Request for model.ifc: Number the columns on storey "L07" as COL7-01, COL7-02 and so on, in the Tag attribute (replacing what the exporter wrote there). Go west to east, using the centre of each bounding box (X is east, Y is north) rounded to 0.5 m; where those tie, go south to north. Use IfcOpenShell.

First a look at what the model holds.

```python
import ifcopenshell
import ifcopenshell.util.element
import ifcopenshell.util.placement

model = ifcopenshell.open("model.ifc")
print(model.schema)
storey = next(s for s in model.by_type("IfcBuildingStorey") if s.Name == "L07")
columns = [e for e in ifcopenshell.util.element.get_decomposition(storey) if e.is_a("IfcColumn")]
for e in sorted(columns, key=lambda e: e.id()):
    origin = ifcopenshell.util.placement.get_local_placement(e.ObjectPlacement)[:3, 3]
    print(e.id(), e.Tag, e.Name, origin.round(2) + 0.0, sep=" | ")
```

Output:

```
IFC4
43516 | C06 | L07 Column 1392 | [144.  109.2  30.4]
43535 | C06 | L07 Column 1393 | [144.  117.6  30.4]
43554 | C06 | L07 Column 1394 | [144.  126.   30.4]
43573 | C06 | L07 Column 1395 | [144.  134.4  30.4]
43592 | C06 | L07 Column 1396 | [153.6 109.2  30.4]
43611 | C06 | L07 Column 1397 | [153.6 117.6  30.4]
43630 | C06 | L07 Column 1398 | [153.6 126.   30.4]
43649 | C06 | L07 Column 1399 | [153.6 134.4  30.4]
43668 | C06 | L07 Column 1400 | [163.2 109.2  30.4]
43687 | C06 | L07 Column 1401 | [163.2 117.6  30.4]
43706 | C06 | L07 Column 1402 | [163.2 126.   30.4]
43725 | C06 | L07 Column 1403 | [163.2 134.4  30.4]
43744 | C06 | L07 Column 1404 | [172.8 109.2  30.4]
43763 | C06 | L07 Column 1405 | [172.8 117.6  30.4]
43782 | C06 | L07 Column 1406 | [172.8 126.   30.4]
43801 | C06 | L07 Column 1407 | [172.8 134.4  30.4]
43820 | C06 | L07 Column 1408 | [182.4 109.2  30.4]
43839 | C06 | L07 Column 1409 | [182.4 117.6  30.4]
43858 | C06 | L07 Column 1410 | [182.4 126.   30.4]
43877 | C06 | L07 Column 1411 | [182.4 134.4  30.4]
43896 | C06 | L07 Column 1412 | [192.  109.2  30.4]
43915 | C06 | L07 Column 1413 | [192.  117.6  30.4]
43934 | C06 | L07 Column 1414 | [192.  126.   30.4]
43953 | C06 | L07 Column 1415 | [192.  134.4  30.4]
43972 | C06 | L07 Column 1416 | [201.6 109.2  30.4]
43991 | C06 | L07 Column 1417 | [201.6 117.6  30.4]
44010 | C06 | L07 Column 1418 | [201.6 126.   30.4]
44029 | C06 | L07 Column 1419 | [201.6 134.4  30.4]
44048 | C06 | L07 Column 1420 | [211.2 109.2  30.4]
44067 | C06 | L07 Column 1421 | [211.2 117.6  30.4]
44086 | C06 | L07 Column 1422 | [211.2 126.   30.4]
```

```python
import ifcopenshell
import ifcopenshell.geom
import ifcopenshell.util.element
import ifcopenshell.util.shape

model = ifcopenshell.open("model.ifc")
settings = ifcopenshell.geom.settings()
settings.set("use-world-coords", True)


def centre(element):
    shape = ifcopenshell.geom.create_shape(settings, element)
    return ifcopenshell.util.shape.get_bbox_centroid(shape.geometry)


storey = next(s for s in model.by_type("IfcBuildingStorey") if s.Name == "L07")
columns = [e for e in ifcopenshell.util.element.get_decomposition(storey) if e.is_a("IfcColumn")]

# Insertion points can sit at a corner or the storey origin, so sort by the geometry (in metres).
centres = {e: centre(e) for e in columns}
columns.sort(key=lambda e: (round(centres[e][0] / 0.5), centres[e][1]))

for i, e in enumerate(columns, start=1):
    number = f"COL7-{i:02d}"
    e.Tag = number
    print(e.id(), number)

model.write("model-out.ifc")
```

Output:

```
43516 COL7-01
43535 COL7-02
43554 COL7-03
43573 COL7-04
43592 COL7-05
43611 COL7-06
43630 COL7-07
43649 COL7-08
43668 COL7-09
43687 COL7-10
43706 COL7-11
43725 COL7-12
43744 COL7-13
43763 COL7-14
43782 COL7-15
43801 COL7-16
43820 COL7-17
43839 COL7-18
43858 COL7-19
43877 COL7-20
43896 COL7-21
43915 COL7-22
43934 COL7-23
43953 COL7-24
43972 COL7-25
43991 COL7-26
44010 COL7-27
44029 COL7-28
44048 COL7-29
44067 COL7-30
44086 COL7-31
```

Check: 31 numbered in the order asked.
